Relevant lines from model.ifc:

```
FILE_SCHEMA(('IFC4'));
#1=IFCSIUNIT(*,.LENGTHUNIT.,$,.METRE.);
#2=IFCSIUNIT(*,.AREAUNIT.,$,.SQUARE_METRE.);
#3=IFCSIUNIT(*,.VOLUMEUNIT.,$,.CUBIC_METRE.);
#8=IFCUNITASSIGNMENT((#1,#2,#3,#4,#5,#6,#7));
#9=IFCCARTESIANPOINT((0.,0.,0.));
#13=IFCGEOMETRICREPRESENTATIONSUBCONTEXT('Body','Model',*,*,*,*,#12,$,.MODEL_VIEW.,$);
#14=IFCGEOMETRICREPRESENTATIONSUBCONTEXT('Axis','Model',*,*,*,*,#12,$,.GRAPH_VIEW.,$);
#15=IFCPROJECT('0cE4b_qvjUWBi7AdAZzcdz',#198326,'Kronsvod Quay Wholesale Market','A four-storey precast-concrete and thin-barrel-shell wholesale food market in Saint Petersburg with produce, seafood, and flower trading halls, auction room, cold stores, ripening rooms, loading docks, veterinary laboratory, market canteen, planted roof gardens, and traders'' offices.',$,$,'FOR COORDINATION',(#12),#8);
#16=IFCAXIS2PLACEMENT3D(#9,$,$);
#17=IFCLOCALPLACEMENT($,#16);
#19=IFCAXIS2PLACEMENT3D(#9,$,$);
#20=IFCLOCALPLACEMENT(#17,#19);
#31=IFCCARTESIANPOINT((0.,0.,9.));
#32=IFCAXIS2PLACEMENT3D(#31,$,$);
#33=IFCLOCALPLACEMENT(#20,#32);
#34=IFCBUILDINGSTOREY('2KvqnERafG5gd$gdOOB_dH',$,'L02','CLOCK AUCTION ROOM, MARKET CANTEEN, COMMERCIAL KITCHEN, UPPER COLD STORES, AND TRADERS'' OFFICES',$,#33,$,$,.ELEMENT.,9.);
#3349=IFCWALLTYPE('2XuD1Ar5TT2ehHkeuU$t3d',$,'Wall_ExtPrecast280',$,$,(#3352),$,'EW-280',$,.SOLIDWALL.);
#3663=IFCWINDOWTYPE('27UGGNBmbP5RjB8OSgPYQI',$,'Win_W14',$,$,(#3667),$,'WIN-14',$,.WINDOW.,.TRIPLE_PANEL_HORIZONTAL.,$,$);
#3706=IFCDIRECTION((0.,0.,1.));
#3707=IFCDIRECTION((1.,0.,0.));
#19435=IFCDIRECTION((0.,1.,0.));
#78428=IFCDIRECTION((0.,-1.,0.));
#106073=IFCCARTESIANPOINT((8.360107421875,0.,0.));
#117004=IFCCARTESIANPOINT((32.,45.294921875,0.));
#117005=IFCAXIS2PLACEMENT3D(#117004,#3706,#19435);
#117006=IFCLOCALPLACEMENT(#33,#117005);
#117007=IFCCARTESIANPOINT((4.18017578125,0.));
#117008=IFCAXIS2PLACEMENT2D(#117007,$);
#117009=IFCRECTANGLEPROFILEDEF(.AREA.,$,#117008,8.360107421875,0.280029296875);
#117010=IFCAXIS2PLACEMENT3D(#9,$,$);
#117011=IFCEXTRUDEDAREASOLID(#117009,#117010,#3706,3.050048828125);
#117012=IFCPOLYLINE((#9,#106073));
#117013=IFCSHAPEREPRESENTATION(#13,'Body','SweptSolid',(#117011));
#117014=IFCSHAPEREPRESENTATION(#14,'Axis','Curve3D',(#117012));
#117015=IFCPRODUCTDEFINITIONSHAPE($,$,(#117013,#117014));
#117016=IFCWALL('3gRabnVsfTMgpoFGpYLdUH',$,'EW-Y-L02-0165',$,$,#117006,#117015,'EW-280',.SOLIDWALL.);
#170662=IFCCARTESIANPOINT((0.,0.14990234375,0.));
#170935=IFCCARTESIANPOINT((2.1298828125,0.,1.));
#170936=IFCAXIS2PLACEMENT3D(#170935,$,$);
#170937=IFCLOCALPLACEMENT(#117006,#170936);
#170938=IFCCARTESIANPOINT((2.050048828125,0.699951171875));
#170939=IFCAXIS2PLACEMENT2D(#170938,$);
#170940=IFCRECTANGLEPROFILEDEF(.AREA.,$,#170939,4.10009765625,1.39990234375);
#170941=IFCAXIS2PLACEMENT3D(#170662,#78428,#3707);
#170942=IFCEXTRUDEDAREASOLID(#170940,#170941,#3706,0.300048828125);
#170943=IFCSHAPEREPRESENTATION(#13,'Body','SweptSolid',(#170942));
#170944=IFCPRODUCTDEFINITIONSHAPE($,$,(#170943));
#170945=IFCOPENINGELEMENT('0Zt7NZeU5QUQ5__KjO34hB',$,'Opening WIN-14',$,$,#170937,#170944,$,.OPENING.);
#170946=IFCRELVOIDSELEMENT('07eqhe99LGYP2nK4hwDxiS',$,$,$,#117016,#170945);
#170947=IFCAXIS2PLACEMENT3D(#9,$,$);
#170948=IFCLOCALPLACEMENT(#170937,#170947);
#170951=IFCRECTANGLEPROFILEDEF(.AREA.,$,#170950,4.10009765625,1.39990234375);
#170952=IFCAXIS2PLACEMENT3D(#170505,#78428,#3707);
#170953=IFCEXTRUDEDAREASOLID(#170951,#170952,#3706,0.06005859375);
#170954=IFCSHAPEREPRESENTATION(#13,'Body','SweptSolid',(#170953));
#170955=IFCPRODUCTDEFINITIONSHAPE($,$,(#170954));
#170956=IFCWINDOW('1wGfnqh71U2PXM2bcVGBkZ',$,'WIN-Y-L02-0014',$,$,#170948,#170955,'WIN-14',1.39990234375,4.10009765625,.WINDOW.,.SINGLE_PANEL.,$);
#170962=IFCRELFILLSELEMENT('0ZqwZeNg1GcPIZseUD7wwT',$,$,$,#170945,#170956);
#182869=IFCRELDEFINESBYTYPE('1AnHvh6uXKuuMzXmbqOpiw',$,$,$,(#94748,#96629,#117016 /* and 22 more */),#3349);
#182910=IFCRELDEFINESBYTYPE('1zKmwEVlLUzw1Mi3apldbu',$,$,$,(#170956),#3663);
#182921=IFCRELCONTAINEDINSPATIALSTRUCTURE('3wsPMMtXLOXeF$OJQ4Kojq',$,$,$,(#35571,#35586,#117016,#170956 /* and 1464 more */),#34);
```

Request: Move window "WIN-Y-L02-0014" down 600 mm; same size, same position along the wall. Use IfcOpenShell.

```python
import numpy as np
import ifcopenshell
import ifcopenshell.api.geometry
import ifcopenshell.util.placement
import ifcopenshell.util.unit

model = ifcopenshell.open("model.ifc")
unit_scale = ifcopenshell.util.unit.calculate_unit_scale(model)

window = model.by_guid("1wGfnqh71U2PXM2bcVGBkZ")
opening = window.FillsVoids[0].RelatingOpeningElement
dz = -0.6 / unit_scale

shift = np.array([0.0, 0.0, dz])
# The window is placed relative to its opening, so it follows when the opening moves.
matrix = ifcopenshell.util.placement.get_local_placement(opening.ObjectPlacement)
matrix[:3, 3] += shift
ifcopenshell.api.geometry.edit_object_placement(
    model, product=opening, matrix=matrix, is_si=False, should_transform_children=True
)

print(f"moved by {dz * unit_scale:+.3f} m")

model.write("model_edited.ifc")
```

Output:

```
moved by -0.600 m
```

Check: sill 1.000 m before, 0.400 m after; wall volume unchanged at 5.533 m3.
